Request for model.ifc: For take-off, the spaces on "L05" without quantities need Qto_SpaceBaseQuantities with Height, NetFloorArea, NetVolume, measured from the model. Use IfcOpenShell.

First a look at what the model holds.

```python
import ifcopenshell
import ifcopenshell.util.element
import ifcopenshell.util.unit

model = ifcopenshell.open("model.ifc")
print(model.schema)
for unit_type in ("LENGTHUNIT", "AREAUNIT", "VOLUMEUNIT"):
    print(unit_type, ifcopenshell.util.unit.calculate_unit_scale(model, unit_type))
storey = next(s for s in model.by_type("IfcBuildingStorey") if s.Name == "L05")
spaces = [e for e in ifcopenshell.util.element.get_decomposition(storey) if e.is_a("IfcSpace")]
for e in sorted(spaces, key=lambda e: e.id()):
    print(e.id(), e.is_a(), e.Name, list(ifcopenshell.util.element.get_psets(e, qtos_only=True)), sep=" | ")
```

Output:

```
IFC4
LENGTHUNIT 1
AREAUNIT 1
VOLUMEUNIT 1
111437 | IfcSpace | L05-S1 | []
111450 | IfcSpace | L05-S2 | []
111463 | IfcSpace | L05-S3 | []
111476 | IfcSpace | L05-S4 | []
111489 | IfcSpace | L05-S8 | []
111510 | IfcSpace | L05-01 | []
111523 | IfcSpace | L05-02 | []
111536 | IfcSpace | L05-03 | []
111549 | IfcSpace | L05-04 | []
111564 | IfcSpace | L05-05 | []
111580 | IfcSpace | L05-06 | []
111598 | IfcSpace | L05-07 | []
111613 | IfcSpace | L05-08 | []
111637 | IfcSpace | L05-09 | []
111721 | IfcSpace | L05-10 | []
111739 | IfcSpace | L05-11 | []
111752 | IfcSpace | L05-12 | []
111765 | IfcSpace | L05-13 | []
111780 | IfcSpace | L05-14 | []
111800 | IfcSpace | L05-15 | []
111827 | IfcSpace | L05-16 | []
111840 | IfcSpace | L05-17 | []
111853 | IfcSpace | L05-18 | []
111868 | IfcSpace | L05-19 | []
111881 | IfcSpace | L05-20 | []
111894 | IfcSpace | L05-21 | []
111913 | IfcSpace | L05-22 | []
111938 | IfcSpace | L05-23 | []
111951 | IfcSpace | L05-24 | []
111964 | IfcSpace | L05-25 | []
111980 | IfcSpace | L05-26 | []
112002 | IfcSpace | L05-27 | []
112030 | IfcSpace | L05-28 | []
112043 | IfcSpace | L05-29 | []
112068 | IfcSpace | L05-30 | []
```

```python
import ifcopenshell
import ifcopenshell.api.pset
import ifcopenshell.geom
import ifcopenshell.util.element
import ifcopenshell.util.shape
import ifcopenshell.util.unit

model = ifcopenshell.open("model.ifc")
unit_scale = ifcopenshell.util.unit.calculate_unit_scale(model)
area_scale = ifcopenshell.util.unit.calculate_unit_scale(model, "AREAUNIT")
volume_scale = ifcopenshell.util.unit.calculate_unit_scale(model, "VOLUMEUNIT")
settings = ifcopenshell.geom.settings()

storey = next(s for s in model.by_type("IfcBuildingStorey") if s.Name == "L05")
spaces = [e for e in ifcopenshell.util.element.get_decomposition(storey) if e.is_a("IfcSpace")]

for e in sorted(spaces, key=lambda e: e.id()):
    if ifcopenshell.util.element.get_psets(e, qtos_only=True, should_inherit=False):
        continue
    # Geometry comes back in metres, in the element's own axes.
    shape = ifcopenshell.geom.create_shape(settings, e)
    values = {
        "Height": ifcopenshell.util.shape.get_z(shape.geometry) / unit_scale,
        "NetFloorArea": ifcopenshell.util.shape.get_footprint_area(shape.geometry) / area_scale,
        "NetVolume": ifcopenshell.util.shape.get_volume(shape.geometry) / volume_scale,
    }
    qto = ifcopenshell.api.pset.add_qto(model, product=e, name="Qto_SpaceBaseQuantities")
    ifcopenshell.api.pset.edit_qto(model, qto=qto, properties=values)
    print(e.id(), {k: round(v, 3) for k, v in values.items()})

model.write("model-out.ifc")
```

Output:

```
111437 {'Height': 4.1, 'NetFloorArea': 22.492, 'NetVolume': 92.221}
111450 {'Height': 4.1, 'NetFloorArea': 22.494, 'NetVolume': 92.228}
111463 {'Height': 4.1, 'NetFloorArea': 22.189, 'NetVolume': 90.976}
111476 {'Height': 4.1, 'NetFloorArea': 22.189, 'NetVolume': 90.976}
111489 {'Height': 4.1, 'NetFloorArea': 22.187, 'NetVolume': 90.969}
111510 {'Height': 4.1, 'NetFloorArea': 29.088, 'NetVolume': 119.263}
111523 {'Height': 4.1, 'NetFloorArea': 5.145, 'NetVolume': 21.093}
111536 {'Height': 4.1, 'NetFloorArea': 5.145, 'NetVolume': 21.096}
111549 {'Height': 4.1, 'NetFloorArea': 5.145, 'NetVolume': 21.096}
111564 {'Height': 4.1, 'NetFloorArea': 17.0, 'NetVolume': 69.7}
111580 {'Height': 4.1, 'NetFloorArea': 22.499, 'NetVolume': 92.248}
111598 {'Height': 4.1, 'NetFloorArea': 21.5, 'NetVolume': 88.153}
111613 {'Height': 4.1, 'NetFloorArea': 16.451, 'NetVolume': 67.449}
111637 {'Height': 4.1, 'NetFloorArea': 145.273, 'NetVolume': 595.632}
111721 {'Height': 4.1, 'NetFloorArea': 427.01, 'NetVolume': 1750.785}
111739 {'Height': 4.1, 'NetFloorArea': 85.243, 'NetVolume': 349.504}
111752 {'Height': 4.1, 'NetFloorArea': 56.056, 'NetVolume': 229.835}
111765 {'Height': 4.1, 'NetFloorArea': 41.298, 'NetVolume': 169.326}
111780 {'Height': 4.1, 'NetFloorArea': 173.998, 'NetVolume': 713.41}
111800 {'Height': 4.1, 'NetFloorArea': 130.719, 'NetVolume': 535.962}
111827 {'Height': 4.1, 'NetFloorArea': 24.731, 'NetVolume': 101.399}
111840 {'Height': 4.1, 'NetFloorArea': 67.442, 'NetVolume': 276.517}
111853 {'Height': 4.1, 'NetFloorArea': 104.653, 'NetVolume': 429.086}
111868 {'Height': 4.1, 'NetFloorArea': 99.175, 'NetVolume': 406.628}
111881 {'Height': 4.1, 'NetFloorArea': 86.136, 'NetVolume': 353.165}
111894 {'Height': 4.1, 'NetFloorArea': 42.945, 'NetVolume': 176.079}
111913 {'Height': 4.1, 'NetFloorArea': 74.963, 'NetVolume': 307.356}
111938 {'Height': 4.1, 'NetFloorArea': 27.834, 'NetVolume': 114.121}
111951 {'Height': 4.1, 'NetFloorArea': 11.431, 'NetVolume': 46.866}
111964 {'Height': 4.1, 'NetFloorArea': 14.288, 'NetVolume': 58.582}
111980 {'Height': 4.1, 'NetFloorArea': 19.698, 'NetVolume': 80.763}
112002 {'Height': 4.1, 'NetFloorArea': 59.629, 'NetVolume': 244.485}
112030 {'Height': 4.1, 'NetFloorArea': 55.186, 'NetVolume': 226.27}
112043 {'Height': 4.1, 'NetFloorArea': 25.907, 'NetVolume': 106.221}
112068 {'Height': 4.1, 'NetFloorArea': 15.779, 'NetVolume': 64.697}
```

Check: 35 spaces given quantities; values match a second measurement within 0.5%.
